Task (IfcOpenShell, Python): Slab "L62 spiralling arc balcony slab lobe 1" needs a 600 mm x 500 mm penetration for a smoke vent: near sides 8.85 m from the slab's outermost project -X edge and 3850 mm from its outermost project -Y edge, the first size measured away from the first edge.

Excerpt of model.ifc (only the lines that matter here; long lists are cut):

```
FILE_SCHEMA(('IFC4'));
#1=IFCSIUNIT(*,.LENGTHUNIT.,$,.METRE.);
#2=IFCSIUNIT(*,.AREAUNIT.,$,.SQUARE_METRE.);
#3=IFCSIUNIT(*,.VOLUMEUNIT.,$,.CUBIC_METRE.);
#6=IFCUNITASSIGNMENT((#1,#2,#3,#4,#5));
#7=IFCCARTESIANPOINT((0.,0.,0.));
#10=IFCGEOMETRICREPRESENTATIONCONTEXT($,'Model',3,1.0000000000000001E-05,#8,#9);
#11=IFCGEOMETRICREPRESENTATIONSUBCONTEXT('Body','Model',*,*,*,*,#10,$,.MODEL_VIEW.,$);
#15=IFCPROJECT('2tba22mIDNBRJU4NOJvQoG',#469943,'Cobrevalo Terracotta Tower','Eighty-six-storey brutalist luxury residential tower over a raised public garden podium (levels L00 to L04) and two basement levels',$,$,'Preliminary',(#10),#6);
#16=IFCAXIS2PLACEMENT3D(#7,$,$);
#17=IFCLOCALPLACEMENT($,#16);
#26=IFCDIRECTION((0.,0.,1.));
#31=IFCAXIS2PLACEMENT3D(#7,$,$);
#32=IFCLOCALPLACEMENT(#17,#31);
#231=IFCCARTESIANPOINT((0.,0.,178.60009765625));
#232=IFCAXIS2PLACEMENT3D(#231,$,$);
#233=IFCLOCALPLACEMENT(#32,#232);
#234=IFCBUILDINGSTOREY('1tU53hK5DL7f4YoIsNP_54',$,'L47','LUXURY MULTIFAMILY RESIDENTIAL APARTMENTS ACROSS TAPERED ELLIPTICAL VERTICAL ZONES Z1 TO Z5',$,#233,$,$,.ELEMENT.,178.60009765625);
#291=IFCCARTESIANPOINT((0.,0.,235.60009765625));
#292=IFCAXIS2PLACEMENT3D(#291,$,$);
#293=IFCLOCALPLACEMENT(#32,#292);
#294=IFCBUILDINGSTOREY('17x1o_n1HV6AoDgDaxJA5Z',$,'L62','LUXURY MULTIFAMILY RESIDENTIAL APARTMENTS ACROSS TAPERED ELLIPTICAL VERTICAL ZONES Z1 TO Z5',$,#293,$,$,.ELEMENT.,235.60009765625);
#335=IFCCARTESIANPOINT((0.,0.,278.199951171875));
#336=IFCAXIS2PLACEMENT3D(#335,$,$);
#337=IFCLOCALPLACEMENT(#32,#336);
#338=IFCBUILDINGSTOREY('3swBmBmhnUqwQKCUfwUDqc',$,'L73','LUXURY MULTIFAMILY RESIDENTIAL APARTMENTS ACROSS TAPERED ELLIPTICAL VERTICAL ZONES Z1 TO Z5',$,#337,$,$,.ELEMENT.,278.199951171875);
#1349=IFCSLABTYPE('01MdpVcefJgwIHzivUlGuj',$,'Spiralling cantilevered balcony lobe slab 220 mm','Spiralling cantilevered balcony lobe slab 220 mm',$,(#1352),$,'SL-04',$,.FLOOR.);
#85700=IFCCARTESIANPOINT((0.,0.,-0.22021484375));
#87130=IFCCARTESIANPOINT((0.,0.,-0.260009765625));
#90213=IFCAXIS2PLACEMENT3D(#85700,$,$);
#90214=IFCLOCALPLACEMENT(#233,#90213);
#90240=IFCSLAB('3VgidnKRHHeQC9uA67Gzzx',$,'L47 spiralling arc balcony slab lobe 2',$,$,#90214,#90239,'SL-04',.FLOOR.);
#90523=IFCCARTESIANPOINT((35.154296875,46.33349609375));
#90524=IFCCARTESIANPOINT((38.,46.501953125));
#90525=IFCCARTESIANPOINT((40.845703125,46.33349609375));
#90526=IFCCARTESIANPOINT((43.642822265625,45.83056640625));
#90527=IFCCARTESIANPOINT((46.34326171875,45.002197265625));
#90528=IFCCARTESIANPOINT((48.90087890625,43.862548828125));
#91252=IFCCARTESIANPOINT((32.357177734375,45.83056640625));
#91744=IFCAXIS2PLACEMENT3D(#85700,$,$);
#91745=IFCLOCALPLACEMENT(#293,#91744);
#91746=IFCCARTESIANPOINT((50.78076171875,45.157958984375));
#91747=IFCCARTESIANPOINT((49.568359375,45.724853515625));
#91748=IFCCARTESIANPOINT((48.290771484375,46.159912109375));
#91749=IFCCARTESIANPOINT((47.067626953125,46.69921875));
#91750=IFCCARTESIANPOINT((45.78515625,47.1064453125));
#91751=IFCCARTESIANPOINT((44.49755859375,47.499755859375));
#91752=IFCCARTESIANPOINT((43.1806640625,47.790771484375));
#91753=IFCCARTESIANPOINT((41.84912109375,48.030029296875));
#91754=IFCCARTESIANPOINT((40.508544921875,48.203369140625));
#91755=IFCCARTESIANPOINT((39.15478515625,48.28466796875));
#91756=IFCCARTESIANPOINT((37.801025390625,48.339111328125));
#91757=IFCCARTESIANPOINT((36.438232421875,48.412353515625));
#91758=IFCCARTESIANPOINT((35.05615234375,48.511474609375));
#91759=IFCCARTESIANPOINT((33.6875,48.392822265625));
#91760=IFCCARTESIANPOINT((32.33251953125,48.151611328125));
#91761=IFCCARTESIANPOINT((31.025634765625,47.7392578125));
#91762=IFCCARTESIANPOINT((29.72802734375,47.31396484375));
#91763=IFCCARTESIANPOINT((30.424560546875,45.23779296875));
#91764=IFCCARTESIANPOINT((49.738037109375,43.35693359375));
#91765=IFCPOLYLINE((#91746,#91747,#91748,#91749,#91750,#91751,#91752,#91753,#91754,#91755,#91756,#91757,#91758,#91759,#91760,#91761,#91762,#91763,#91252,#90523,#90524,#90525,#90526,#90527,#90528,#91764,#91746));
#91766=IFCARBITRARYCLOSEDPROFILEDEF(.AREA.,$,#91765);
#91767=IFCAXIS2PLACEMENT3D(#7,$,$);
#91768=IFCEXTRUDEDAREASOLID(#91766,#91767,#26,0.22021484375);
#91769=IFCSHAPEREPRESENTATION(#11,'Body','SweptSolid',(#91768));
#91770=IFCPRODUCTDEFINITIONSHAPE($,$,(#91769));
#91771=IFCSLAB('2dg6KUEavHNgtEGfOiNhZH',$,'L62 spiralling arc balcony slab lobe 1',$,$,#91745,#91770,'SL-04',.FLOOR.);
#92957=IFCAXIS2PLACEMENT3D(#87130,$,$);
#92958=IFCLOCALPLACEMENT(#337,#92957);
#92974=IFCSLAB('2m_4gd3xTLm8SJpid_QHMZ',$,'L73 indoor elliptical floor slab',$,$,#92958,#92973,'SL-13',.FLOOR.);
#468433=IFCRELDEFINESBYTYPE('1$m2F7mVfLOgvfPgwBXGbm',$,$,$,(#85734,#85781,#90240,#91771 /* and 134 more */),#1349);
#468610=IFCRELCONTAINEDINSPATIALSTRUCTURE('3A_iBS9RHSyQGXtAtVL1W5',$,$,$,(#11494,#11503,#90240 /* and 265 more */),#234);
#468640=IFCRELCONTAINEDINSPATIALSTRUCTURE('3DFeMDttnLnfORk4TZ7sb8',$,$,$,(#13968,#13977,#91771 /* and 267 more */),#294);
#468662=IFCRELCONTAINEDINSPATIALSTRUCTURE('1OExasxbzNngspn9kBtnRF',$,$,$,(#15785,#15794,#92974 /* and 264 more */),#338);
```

```python
import numpy as np
import ifcopenshell
import ifcopenshell.api.feature
import ifcopenshell.api.geometry
import ifcopenshell.api.root
import ifcopenshell.geom
import ifcopenshell.util.placement
import ifcopenshell.util.representation
import ifcopenshell.util.shape
import ifcopenshell.util.unit

model = ifcopenshell.open("model.ifc")
unit_scale = ifcopenshell.util.unit.calculate_unit_scale(model)
settings = ifcopenshell.geom.settings()


def volume(element):
    """Net volume in cubic metres, openings subtracted."""
    shape = ifcopenshell.geom.create_shape(settings, element)
    return ifcopenshell.util.shape.get_volume(shape.geometry)


slab = model.by_guid("2dg6KUEavHNgtEGfOiNhZH")
before = volume(slab)

# Extent in the slab's own axes, in metres. The edges named are its -X and -Y sides.
slab_shape = ifcopenshell.geom.create_shape(settings, slab)
vertices = ifcopenshell.util.shape.get_vertices(slab_shape.geometry)
x_min, y_min, bottom = vertices.min(axis=0)
top = vertices[:, 2].max()

opening = ifcopenshell.api.root.create_entity(model, ifc_class="IfcOpeningElement", name="Smoke vent opening", predefined_type="OPENING")
context = ifcopenshell.util.representation.get_context(model, "Model", "Body", "MODEL_VIEW")
width, depth = 0.6, 0.5
outline = [(0.0, 0.0), (width, 0.0), (width, depth), (0.0, depth), (0.0, 0.0)]
# Overshoot both faces by 50 mm so the cut is clean.
shape = ifcopenshell.api.geometry.add_slab_representation(
    model, context=context, depth=top - bottom + 0.1, polyline=outline
)
ifcopenshell.api.geometry.assign_representation(model, product=opening, representation=shape)

matrix = ifcopenshell.util.placement.get_local_placement(slab.ObjectPlacement)
matrix[:, 3] = matrix @ np.append(np.array([x_min + 8.85, y_min + 3.85, bottom - 0.05]) / unit_scale, 1.0)
ifcopenshell.api.geometry.edit_object_placement(model, product=opening, matrix=matrix, is_si=False)
ifcopenshell.api.feature.add_feature(model, feature=opening, element=slab)

after = volume(slab)

print(f"slab volume {before:.3f} -> {after:.3f} m3")

model.write("model-out.ifc")
```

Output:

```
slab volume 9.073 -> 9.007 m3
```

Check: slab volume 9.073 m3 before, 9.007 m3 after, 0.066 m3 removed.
